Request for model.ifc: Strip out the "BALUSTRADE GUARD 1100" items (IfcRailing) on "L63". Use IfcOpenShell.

First a look at what the model holds.

```python
import ifcopenshell
import ifcopenshell.util.element

model = ifcopenshell.open("model.ifc")
print(model.schema)
storey = next(s for s in model.by_type("IfcBuildingStorey") if s.Name == "L63")
railings = [e for e in ifcopenshell.util.element.get_decomposition(storey) if e.is_a("IfcRailing")]
seen = {}
for e in railings:
    element_type = ifcopenshell.util.element.get_type(e)
    name = element_type.Name if element_type not in (None, e) else None
    seen[name] = seen.get(name, 0) + 1
for name, count in sorted(seen.items(), key=str):
    print(count, "x", name)
```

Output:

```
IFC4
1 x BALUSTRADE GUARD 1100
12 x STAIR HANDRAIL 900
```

```python
import ifcopenshell
import ifcopenshell.api.root
import ifcopenshell.util.element

model = ifcopenshell.open("model.ifc")

storey = next(s for s in model.by_type("IfcBuildingStorey") if s.Name == "L63")
railings = [e for e in ifcopenshell.util.element.get_decomposition(storey) if e.is_a("IfcRailing")]
targets = [e for e in railings if (t := ifcopenshell.util.element.get_type(e)) not in (None, e) and t.Name == "BALUSTRADE GUARD 1100"]

for e in targets:
    ifcopenshell.api.root.remove_product(model, product=e)
print(len(targets), "removed")

model.write("model_edited.ifc")
```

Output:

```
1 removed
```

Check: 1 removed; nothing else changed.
